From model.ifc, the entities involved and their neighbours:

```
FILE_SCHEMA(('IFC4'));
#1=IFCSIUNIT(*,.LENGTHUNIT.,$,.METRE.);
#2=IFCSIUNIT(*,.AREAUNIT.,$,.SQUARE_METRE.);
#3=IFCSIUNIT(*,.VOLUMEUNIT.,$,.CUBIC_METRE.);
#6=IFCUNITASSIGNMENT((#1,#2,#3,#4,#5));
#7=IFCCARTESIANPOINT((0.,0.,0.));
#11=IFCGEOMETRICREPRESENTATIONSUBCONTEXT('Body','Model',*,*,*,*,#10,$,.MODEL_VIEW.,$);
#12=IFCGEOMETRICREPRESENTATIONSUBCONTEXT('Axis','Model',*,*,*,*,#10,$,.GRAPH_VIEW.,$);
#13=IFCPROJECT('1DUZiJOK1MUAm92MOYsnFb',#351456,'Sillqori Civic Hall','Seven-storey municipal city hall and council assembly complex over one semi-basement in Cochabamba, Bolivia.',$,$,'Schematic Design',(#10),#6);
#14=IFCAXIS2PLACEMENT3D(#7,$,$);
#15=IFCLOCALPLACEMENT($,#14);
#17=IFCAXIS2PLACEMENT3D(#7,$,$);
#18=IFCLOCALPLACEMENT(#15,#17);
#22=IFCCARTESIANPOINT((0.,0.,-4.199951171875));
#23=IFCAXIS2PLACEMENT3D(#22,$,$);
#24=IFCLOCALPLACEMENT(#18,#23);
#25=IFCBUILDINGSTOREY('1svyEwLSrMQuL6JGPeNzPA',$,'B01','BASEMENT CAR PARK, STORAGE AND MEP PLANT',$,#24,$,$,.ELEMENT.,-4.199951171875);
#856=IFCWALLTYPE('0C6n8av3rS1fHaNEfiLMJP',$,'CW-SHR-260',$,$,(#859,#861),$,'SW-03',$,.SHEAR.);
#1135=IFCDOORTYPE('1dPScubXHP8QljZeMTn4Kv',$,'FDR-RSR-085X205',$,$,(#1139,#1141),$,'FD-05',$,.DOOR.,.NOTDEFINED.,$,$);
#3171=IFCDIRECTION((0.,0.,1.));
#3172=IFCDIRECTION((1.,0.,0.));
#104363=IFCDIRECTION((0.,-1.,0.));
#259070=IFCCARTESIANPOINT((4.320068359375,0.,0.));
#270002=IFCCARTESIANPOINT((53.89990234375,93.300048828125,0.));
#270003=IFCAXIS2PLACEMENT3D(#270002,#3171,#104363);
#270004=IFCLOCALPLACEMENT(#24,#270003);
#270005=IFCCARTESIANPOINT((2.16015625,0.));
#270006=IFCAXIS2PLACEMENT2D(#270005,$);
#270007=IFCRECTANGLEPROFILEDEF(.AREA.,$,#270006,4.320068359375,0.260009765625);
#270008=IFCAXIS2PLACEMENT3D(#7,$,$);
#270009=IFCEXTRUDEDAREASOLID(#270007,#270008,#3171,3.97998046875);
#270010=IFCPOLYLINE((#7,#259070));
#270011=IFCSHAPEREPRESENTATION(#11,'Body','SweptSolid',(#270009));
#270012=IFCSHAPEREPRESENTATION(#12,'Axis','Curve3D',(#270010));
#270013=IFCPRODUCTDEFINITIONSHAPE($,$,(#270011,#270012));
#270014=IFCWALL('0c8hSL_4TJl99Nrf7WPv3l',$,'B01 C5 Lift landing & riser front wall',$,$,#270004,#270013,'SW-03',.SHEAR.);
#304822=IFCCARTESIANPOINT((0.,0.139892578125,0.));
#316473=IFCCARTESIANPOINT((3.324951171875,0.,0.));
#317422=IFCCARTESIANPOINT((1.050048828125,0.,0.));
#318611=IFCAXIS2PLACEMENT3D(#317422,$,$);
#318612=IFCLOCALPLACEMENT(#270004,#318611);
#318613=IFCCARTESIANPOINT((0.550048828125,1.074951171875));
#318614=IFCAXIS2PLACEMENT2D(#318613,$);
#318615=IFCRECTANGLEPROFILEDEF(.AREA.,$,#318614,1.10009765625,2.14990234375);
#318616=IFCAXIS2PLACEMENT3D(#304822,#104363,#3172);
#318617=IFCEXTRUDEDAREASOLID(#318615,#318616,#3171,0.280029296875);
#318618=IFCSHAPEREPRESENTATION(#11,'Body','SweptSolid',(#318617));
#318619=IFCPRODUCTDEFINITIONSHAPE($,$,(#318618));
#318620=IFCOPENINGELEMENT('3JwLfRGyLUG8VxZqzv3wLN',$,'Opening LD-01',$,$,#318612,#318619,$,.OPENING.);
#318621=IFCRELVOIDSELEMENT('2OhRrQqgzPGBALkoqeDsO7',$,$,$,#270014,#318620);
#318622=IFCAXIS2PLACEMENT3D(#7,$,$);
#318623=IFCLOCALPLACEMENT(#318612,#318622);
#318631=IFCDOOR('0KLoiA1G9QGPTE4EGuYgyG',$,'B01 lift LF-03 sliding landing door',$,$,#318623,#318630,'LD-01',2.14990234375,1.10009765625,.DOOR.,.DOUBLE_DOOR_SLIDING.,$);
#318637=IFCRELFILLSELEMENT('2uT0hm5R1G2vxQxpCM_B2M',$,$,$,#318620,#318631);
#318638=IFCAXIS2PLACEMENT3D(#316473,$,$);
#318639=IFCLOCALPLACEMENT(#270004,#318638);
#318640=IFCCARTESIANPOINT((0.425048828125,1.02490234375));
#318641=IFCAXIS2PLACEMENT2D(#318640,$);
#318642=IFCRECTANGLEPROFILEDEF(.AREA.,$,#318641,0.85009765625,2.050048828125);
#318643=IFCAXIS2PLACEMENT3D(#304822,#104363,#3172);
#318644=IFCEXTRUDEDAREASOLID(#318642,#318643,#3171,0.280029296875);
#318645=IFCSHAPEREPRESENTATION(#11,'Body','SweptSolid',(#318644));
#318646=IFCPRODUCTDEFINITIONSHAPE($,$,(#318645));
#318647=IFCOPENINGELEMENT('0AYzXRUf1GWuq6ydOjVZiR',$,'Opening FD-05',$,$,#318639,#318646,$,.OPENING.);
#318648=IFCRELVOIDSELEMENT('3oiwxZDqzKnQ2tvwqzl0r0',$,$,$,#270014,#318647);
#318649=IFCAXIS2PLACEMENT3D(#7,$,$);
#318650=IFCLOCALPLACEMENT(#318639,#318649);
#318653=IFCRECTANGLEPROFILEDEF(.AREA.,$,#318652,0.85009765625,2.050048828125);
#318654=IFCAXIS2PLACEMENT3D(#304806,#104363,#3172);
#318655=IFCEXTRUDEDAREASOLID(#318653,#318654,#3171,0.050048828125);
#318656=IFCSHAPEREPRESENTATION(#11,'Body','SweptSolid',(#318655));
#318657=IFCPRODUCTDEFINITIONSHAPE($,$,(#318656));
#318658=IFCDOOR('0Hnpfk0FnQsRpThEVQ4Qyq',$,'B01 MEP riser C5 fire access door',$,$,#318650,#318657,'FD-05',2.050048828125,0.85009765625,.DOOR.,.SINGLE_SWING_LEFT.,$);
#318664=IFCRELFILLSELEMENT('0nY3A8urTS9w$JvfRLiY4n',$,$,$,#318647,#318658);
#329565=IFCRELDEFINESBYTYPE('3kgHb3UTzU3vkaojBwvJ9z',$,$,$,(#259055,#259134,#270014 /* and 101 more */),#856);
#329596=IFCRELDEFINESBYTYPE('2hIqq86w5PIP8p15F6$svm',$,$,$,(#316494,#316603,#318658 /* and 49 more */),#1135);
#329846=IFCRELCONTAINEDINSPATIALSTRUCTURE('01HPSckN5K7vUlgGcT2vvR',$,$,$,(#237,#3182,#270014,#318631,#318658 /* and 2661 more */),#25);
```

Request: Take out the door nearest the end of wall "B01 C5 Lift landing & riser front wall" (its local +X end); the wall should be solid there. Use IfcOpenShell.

```python
import ifcopenshell
import ifcopenshell.api.feature
import ifcopenshell.api.root
import ifcopenshell.geom
import ifcopenshell.util.shape

model = ifcopenshell.open("model.ifc")
settings = ifcopenshell.geom.settings()


def volume(element):
    """Net volume in cubic metres, openings subtracted."""
    shape = ifcopenshell.geom.create_shape(settings, element)
    return ifcopenshell.util.shape.get_volume(shape.geometry)


door = model.by_id(318658)
opening = door.FillsVoids[0].RelatingOpeningElement
wall = opening.VoidsElements[0].RelatingBuildingElement
before = volume(wall)

ifcopenshell.api.root.remove_product(model, product=door)
ifcopenshell.api.feature.remove_feature(model, feature=opening)

after = volume(wall)

print(f"wall volume {before:.3f} -> {after:.3f} m3")

model.write("model_updated.ifc")
```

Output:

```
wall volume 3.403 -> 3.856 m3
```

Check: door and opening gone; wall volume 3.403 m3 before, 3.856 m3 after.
